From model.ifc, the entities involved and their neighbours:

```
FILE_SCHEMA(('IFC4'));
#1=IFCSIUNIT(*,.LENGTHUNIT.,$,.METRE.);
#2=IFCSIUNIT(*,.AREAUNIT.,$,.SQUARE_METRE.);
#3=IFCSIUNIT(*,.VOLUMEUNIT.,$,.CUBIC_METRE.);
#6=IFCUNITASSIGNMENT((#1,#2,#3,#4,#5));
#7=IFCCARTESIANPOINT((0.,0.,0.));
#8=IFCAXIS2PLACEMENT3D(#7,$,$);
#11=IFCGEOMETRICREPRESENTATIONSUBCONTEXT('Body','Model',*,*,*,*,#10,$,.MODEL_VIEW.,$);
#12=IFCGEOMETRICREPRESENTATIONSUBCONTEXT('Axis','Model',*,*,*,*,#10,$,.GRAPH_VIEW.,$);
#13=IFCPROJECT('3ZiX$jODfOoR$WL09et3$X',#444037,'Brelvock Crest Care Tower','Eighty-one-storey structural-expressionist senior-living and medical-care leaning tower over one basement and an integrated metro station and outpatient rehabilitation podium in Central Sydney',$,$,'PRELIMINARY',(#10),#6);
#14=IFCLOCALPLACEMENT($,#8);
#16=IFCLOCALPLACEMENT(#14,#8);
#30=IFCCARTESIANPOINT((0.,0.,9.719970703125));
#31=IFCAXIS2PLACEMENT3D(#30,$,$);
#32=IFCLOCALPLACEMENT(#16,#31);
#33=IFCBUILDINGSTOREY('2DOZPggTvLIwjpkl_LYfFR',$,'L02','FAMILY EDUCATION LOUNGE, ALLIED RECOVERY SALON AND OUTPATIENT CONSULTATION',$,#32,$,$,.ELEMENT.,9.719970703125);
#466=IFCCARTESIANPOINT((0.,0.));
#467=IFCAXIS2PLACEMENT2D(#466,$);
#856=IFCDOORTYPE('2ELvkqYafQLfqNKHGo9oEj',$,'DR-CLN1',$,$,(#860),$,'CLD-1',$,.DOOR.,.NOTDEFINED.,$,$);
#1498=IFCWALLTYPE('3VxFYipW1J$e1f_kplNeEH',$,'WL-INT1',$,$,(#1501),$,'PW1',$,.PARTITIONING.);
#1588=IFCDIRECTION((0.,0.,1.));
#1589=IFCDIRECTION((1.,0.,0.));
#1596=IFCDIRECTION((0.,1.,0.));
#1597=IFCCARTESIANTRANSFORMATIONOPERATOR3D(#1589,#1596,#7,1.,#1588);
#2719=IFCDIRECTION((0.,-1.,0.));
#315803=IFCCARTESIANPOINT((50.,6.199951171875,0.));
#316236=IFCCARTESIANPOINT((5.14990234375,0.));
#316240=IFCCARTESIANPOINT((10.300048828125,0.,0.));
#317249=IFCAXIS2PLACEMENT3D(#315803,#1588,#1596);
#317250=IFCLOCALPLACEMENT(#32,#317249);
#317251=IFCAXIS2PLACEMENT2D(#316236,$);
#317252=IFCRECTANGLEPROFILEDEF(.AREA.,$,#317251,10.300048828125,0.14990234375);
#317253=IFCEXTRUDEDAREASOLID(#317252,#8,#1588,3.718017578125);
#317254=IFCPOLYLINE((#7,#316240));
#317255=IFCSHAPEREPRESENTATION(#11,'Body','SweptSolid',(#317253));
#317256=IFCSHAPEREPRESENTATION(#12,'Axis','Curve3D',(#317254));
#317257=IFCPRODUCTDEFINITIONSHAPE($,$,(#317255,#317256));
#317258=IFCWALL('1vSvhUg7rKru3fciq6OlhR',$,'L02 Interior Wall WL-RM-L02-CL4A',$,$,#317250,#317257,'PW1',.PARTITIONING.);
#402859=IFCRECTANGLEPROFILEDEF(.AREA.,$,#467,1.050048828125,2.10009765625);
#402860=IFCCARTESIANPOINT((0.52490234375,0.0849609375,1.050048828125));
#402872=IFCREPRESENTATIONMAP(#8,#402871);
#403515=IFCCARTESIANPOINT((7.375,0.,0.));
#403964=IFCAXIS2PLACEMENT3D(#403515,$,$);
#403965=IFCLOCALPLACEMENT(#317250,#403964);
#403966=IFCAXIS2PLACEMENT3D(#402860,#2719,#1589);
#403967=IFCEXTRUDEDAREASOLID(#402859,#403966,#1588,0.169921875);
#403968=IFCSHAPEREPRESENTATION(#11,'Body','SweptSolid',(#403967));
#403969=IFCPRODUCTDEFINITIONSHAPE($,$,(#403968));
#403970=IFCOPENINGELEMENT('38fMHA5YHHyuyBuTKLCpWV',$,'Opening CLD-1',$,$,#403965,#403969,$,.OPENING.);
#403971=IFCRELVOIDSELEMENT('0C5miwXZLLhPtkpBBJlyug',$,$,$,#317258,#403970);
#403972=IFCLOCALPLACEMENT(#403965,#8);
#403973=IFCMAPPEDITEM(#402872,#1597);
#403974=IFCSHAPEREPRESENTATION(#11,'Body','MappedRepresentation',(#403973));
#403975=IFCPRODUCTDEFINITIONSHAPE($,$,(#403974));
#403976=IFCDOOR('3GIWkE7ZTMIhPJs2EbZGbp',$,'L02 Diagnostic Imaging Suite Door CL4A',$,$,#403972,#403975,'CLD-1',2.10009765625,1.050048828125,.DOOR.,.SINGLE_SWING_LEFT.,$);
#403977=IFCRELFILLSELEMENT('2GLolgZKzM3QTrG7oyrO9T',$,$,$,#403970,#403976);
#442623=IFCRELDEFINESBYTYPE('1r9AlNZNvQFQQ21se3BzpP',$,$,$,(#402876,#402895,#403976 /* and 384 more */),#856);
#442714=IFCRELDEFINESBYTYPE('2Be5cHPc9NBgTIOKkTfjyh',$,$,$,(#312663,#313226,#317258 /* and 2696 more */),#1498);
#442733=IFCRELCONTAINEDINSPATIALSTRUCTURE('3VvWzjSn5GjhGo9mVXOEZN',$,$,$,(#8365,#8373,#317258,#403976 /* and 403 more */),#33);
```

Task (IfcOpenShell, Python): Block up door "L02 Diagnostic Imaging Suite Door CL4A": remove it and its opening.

```python
import ifcopenshell
import ifcopenshell.api.feature
import ifcopenshell.api.root
import ifcopenshell.geom
import ifcopenshell.util.shape

model = ifcopenshell.open("model.ifc")
settings = ifcopenshell.geom.settings()


def volume(element):
    """Net volume in cubic metres, openings subtracted."""
    shape = ifcopenshell.geom.create_shape(settings, element)
    return ifcopenshell.util.shape.get_volume(shape.geometry)


door = model.by_id(403976)
opening = door.FillsVoids[0].RelatingOpeningElement
wall = opening.VoidsElements[0].RelatingBuildingElement
before = volume(wall)

ifcopenshell.api.root.remove_product(model, product=door)
ifcopenshell.api.feature.remove_feature(model, feature=opening)

after = volume(wall)

print(f"wall volume {before:.3f} -> {after:.3f} m3")

model.write("model_rev.ifc")
```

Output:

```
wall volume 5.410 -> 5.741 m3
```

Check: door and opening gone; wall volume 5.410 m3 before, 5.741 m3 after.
